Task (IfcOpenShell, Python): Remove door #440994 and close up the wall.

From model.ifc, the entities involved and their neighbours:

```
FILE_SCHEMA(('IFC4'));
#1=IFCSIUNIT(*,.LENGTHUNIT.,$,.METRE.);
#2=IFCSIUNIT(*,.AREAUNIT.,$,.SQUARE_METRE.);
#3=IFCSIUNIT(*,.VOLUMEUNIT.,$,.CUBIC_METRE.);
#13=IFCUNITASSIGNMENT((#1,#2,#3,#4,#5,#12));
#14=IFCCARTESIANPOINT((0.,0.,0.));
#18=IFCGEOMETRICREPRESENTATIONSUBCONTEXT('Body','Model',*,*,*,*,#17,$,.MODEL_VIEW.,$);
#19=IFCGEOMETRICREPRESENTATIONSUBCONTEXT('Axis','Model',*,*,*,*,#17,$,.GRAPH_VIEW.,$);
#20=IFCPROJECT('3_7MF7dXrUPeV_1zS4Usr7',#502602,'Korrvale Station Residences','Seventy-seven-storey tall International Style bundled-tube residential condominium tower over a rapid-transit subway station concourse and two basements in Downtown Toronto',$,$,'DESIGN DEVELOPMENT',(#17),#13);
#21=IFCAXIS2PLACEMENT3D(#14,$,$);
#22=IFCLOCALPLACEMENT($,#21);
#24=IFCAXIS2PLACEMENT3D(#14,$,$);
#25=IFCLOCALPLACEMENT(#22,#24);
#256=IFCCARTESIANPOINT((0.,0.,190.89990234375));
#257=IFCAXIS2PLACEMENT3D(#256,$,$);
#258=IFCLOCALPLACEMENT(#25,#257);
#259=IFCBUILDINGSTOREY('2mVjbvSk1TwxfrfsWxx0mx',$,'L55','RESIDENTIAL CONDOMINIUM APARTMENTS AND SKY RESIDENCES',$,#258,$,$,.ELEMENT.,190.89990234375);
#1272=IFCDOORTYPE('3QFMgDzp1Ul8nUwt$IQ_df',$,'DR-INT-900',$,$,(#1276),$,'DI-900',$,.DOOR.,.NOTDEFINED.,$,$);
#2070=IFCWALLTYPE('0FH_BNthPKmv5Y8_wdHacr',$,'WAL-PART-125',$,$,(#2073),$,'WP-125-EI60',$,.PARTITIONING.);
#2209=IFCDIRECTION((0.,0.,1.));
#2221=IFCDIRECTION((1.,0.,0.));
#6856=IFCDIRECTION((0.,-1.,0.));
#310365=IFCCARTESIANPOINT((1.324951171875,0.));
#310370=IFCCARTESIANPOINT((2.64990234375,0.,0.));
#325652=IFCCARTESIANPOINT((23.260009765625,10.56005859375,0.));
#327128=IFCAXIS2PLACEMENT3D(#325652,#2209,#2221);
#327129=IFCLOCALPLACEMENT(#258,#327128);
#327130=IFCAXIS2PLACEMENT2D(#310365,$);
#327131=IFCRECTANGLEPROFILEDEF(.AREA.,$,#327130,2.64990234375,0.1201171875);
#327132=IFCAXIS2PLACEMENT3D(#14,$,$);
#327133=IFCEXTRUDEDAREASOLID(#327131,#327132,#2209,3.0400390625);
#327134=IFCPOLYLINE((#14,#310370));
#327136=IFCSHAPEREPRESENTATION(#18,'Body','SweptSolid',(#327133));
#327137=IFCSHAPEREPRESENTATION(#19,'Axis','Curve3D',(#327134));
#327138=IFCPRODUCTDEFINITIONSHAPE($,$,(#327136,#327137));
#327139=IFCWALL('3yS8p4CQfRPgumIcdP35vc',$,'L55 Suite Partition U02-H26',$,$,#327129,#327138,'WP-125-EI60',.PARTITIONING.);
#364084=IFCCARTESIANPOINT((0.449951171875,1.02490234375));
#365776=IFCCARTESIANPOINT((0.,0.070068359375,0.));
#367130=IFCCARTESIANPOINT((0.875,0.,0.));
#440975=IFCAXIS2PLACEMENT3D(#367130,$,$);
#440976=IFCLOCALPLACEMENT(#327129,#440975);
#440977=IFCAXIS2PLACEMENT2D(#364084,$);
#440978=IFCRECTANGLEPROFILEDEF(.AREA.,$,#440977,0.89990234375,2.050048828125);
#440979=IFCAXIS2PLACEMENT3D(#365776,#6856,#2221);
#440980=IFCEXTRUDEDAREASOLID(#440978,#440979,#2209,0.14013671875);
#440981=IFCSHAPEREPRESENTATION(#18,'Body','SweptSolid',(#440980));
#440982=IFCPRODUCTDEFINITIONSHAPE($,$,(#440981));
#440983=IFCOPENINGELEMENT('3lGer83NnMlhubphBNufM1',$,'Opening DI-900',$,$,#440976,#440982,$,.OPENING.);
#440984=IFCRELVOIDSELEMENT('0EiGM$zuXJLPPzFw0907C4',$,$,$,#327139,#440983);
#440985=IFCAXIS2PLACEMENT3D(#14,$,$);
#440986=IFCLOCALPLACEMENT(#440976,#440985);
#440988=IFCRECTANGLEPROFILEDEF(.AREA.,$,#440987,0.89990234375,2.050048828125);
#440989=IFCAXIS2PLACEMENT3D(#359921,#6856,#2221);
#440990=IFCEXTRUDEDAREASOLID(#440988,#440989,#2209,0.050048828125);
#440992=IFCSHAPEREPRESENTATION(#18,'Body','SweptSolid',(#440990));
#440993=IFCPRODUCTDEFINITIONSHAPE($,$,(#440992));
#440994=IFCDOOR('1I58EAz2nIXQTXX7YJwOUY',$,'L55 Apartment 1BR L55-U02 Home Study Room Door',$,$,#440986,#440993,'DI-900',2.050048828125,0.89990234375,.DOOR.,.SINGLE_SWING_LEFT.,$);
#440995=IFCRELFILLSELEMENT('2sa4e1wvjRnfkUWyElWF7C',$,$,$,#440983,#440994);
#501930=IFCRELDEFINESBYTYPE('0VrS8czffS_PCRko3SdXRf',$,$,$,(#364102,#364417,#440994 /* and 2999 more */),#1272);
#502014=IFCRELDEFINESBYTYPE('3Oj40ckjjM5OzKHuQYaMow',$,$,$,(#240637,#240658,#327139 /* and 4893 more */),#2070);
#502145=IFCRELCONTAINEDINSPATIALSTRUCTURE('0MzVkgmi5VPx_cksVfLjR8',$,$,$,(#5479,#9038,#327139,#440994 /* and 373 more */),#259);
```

```python
import ifcopenshell
import ifcopenshell.api.feature
import ifcopenshell.api.root
import ifcopenshell.geom
import ifcopenshell.util.shape

model = ifcopenshell.open("model.ifc")
settings = ifcopenshell.geom.settings()


def volume(element):
    """Net volume in cubic metres, openings subtracted."""
    shape = ifcopenshell.geom.create_shape(settings, element)
    return ifcopenshell.util.shape.get_volume(shape.geometry)


door = model.by_id(440994)
opening = door.FillsVoids[0].RelatingOpeningElement
wall = opening.VoidsElements[0].RelatingBuildingElement
before = volume(wall)

ifcopenshell.api.root.remove_product(model, product=door)
ifcopenshell.api.feature.remove_feature(model, feature=opening)

after = volume(wall)

print(f"wall volume {before:.3f} -> {after:.3f} m3")

model.write("model_edited.ifc")
```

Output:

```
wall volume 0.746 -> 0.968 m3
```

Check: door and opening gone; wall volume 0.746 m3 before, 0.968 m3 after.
